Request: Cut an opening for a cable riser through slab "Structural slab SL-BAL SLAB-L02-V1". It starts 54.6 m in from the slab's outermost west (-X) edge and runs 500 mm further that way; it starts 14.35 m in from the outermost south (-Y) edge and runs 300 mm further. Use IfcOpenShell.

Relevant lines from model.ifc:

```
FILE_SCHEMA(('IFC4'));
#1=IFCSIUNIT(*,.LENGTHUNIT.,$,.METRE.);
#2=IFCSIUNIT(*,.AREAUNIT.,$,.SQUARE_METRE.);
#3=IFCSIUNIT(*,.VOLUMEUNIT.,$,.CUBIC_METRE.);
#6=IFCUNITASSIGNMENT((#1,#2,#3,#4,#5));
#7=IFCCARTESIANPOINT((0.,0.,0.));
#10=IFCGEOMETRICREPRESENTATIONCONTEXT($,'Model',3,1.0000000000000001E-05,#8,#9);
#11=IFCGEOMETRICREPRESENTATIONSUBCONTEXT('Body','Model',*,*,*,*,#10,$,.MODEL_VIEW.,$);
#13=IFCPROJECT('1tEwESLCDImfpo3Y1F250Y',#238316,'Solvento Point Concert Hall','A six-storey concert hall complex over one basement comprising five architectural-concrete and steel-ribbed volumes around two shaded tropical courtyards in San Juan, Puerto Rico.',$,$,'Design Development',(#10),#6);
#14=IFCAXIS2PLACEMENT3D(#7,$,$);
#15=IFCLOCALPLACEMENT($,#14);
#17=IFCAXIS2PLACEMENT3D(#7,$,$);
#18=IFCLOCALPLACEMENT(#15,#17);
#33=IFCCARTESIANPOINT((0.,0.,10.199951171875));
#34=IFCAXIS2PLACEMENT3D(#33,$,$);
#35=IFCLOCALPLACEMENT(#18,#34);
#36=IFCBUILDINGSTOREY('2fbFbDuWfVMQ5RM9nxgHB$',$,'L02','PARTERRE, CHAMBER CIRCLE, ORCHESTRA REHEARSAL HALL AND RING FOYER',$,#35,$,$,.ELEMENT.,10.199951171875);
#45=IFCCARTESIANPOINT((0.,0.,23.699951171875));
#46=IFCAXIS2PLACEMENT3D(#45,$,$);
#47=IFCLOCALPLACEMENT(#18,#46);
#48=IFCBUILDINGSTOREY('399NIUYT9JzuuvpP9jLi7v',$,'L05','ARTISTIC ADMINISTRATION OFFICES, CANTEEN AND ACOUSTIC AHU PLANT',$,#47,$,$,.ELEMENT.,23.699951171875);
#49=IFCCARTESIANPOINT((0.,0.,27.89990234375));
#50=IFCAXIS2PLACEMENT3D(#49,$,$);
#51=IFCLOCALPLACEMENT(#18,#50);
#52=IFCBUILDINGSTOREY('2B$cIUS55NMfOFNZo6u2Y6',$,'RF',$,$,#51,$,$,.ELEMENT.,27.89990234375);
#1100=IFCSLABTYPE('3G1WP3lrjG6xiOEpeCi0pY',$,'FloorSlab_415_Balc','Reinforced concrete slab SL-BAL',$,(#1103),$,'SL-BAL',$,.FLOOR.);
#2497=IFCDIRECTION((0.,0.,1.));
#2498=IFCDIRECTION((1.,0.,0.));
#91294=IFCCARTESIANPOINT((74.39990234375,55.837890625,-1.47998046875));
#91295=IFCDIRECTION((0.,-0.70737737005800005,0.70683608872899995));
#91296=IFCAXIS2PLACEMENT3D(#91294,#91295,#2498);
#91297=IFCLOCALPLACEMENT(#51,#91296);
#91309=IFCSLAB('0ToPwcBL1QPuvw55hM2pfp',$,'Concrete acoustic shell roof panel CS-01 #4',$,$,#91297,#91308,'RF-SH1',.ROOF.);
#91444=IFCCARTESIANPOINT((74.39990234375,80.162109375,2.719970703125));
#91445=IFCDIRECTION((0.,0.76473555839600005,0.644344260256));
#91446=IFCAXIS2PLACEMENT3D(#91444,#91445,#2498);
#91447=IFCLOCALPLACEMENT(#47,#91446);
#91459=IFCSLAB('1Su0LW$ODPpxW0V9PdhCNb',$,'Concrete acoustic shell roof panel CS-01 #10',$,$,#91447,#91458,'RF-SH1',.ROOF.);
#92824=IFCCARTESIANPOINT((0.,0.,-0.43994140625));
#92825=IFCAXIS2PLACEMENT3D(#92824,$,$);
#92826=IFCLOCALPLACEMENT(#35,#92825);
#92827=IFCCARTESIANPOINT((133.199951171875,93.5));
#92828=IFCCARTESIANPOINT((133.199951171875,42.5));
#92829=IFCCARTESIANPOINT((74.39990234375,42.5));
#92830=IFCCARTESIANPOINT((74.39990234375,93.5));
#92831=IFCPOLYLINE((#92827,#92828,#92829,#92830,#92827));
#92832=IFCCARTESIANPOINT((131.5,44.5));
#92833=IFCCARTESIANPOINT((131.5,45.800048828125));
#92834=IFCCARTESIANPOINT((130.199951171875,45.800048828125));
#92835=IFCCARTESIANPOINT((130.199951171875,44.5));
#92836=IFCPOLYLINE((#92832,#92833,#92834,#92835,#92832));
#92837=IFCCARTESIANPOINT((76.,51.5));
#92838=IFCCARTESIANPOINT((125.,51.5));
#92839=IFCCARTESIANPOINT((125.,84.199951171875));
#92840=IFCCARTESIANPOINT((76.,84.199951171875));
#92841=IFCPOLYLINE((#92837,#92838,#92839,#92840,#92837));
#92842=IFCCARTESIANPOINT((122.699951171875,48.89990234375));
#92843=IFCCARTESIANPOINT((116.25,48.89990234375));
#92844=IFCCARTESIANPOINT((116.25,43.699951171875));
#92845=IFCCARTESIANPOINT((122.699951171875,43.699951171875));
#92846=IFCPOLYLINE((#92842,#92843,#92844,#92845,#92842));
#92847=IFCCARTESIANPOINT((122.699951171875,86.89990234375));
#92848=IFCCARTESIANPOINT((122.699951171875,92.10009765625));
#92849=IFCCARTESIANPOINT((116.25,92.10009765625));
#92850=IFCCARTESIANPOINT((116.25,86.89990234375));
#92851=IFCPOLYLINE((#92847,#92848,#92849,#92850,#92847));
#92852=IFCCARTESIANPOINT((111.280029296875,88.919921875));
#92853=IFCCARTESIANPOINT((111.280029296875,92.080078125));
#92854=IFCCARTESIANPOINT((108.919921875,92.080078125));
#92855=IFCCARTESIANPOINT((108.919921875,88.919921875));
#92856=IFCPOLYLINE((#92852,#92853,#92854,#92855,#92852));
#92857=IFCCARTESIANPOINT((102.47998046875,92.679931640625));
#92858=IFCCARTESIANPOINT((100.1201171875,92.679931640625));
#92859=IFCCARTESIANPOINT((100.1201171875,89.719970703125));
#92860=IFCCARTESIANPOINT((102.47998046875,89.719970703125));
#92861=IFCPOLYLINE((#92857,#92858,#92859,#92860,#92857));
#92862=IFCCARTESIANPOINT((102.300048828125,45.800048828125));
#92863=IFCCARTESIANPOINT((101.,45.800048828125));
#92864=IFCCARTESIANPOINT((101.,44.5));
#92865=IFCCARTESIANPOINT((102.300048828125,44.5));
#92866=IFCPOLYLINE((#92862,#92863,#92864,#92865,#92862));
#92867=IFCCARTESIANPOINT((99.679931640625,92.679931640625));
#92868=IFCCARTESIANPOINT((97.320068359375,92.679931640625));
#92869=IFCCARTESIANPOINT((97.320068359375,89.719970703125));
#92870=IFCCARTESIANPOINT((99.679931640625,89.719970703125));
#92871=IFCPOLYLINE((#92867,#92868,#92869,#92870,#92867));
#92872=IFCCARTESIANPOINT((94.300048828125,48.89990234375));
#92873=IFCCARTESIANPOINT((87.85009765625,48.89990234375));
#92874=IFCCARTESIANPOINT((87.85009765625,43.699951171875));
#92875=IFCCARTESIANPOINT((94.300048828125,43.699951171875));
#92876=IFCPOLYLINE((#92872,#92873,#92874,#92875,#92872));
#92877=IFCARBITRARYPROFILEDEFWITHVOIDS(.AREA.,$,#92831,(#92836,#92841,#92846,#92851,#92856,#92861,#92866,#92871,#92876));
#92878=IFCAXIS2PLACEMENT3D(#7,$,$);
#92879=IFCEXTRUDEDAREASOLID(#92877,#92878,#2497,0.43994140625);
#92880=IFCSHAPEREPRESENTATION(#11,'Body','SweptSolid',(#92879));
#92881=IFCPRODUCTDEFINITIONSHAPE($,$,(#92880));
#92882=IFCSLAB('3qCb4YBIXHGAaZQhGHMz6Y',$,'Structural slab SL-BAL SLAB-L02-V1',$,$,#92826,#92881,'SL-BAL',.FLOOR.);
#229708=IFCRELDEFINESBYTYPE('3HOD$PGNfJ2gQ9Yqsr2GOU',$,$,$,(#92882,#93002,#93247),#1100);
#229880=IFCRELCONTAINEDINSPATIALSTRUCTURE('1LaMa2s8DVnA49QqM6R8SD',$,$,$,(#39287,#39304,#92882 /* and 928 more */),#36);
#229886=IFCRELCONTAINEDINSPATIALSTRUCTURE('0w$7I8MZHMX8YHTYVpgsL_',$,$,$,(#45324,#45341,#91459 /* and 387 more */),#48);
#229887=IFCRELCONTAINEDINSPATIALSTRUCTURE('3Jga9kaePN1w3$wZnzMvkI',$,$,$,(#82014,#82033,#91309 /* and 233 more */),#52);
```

```python
import numpy as np
import ifcopenshell
import ifcopenshell.api.feature
import ifcopenshell.api.geometry
import ifcopenshell.api.root
import ifcopenshell.geom
import ifcopenshell.util.placement
import ifcopenshell.util.representation
import ifcopenshell.util.shape
import ifcopenshell.util.unit

model = ifcopenshell.open("model.ifc")
unit_scale = ifcopenshell.util.unit.calculate_unit_scale(model)
settings = ifcopenshell.geom.settings()


def volume(element):
    """Net volume in cubic metres, openings subtracted."""
    shape = ifcopenshell.geom.create_shape(settings, element)
    return ifcopenshell.util.shape.get_volume(shape.geometry)


slab = model.by_guid("3qCb4YBIXHGAaZQhGHMz6Y")
before = volume(slab)

# Extent in the slab's own axes, in metres. The edges named are its -X and -Y sides.
slab_shape = ifcopenshell.geom.create_shape(settings, slab)
vertices = ifcopenshell.util.shape.get_vertices(slab_shape.geometry)
x_min, y_min, bottom = vertices.min(axis=0)
top = vertices[:, 2].max()

opening = ifcopenshell.api.root.create_entity(model, ifc_class="IfcOpeningElement", name="Cable riser opening", predefined_type="OPENING")
context = ifcopenshell.util.representation.get_context(model, "Model", "Body", "MODEL_VIEW")
width, depth = 0.5, 0.3
outline = [(0.0, 0.0), (width, 0.0), (width, depth), (0.0, depth), (0.0, 0.0)]
# Overshoot both faces by 50 mm so the cut is clean.
shape = ifcopenshell.api.geometry.add_slab_representation(
    model, context=context, depth=top - bottom + 0.1, polyline=outline
)
ifcopenshell.api.geometry.assign_representation(model, product=opening, representation=shape)

matrix = ifcopenshell.util.placement.get_local_placement(slab.ObjectPlacement)
matrix[:, 3] = matrix @ np.append(np.array([x_min + 54.6, y_min + 14.35, bottom - 0.05]) / unit_scale, 1.0)
ifcopenshell.api.geometry.edit_object_placement(model, product=opening, matrix=matrix, is_si=False)
ifcopenshell.api.feature.add_feature(model, feature=opening, element=slab)

after = volume(slab)

print(f"slab volume {before:.3f} -> {after:.3f} m3")

model.write("model_edited.ifc")
```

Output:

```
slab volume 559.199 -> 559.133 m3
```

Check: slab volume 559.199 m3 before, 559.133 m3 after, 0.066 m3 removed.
